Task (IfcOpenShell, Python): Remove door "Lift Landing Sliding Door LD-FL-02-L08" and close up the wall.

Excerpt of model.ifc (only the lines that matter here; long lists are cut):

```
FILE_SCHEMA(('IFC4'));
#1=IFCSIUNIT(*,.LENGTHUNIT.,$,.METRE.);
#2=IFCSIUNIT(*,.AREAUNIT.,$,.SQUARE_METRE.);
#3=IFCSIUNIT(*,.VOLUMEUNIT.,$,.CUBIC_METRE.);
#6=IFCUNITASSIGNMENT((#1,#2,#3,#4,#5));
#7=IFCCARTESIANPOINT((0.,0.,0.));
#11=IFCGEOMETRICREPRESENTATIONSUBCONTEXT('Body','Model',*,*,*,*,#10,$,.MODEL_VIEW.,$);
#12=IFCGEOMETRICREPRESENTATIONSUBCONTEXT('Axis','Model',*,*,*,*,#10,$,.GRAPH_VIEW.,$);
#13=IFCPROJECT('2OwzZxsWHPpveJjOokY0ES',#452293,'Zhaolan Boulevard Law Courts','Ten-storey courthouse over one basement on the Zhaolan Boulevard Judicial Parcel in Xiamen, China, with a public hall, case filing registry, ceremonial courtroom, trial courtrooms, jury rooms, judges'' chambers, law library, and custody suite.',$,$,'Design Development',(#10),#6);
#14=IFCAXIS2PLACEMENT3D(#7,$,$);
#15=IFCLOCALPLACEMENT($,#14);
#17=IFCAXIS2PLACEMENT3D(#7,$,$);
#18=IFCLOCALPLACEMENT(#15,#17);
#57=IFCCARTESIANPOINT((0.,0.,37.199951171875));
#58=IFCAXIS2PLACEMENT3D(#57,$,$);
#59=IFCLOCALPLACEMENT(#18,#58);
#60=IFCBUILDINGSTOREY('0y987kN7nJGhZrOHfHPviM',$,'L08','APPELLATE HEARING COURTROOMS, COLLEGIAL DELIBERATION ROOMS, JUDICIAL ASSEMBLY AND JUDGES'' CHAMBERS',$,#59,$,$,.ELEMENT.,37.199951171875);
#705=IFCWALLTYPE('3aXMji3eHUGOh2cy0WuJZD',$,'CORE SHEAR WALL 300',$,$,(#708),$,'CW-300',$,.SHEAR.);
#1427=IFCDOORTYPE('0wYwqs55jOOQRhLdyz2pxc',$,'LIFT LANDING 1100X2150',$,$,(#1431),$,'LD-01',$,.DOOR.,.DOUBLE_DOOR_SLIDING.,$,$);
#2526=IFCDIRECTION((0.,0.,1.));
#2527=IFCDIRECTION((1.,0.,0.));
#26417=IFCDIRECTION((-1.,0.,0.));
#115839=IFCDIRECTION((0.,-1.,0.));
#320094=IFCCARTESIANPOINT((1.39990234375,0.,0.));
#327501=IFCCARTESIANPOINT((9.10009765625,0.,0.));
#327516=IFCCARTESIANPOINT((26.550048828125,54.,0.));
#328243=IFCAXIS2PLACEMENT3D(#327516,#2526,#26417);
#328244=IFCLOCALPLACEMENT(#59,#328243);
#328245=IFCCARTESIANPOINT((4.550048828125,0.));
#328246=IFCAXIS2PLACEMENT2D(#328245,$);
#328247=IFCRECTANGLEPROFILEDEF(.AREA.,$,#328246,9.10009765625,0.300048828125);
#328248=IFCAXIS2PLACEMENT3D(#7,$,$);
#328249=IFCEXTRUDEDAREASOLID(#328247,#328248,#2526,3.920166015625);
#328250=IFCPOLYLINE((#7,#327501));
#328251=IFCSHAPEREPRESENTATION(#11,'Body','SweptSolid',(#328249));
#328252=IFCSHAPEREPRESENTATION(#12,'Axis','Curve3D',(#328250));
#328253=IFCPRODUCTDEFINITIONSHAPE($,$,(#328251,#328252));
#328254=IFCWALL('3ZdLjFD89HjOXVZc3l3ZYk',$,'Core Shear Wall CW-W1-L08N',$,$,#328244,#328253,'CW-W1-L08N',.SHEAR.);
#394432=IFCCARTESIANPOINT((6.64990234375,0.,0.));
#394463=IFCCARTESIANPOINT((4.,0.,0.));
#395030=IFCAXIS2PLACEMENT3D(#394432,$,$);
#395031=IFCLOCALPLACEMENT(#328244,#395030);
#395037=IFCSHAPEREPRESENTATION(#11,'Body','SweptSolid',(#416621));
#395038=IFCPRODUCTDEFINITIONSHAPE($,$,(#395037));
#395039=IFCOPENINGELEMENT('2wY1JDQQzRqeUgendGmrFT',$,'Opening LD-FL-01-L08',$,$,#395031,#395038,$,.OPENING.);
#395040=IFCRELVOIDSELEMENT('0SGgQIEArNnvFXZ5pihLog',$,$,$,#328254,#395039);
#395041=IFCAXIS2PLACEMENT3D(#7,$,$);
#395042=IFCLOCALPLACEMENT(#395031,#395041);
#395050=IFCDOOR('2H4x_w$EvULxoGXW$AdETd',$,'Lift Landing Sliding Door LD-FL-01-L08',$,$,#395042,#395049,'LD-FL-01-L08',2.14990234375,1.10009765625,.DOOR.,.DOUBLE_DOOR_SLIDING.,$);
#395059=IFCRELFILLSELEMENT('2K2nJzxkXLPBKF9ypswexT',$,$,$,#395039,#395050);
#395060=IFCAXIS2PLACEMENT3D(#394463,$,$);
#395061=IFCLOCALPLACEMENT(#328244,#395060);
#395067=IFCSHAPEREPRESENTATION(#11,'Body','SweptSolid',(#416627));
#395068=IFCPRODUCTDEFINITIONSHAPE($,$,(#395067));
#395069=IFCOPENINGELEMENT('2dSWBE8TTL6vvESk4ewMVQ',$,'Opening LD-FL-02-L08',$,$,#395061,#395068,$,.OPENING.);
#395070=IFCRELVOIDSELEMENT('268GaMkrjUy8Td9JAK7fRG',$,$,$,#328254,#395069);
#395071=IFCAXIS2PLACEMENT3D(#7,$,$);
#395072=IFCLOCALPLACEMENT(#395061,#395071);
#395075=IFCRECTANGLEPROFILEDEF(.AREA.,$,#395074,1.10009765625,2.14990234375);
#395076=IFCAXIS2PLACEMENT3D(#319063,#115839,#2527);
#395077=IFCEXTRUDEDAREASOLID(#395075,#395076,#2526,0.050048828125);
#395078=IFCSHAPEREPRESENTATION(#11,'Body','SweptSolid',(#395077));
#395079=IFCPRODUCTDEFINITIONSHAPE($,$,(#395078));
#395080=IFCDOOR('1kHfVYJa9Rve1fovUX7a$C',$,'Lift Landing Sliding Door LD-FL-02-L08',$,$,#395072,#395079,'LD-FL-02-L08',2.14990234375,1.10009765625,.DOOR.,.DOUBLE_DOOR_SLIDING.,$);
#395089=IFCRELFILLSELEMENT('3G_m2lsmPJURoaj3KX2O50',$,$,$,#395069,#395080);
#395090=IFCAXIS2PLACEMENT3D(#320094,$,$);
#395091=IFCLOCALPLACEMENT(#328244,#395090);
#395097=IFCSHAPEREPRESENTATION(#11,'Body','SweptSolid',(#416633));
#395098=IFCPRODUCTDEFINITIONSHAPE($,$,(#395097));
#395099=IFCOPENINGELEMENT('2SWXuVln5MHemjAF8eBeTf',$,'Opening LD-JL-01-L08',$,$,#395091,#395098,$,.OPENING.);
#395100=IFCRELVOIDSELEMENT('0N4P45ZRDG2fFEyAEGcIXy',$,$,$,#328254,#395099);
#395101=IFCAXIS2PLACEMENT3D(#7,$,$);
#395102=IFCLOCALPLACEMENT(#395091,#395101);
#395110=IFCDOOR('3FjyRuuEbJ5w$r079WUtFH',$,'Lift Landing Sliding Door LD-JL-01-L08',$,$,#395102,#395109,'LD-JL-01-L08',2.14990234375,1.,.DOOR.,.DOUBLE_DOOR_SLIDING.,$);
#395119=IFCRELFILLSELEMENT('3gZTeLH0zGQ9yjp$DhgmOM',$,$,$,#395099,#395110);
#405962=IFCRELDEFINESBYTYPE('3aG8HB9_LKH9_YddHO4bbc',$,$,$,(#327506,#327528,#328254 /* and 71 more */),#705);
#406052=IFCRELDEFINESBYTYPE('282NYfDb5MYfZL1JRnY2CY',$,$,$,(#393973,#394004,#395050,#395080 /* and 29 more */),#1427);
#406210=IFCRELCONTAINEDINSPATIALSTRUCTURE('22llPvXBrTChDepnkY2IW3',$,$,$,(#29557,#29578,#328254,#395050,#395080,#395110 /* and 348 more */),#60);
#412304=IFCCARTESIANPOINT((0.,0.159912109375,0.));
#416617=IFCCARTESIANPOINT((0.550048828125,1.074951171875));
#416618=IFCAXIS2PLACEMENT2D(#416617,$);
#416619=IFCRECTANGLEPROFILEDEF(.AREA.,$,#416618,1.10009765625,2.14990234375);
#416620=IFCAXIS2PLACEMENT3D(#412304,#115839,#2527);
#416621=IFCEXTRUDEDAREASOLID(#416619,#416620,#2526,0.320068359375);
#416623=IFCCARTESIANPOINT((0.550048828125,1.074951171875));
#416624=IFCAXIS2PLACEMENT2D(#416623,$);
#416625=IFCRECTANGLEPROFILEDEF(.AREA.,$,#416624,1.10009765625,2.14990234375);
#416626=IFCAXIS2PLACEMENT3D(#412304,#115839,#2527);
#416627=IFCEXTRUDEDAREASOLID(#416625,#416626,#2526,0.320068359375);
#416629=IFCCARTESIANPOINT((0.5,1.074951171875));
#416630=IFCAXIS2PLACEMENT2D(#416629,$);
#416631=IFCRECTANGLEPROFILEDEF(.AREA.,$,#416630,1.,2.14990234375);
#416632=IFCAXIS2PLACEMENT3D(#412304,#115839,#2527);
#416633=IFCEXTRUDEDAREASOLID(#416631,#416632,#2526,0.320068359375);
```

```python
import ifcopenshell
import ifcopenshell.api.feature
import ifcopenshell.api.root
import ifcopenshell.geom
import ifcopenshell.util.shape

model = ifcopenshell.open("model.ifc")
settings = ifcopenshell.geom.settings()


def volume(element):
    """Net volume in cubic metres, openings subtracted."""
    shape = ifcopenshell.geom.create_shape(settings, element)
    return ifcopenshell.util.shape.get_volume(shape.geometry)


door = model.by_id(395080)
opening = door.FillsVoids[0].RelatingOpeningElement
wall = opening.VoidsElements[0].RelatingBuildingElement
before = volume(wall)

ifcopenshell.api.root.remove_product(model, product=door)
ifcopenshell.api.feature.remove_feature(model, feature=opening)

after = volume(wall)

print(f"wall volume {before:.3f} -> {after:.3f} m3")

model.write("model_v2.ifc")
```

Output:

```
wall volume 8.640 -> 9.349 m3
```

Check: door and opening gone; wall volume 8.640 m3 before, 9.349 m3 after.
